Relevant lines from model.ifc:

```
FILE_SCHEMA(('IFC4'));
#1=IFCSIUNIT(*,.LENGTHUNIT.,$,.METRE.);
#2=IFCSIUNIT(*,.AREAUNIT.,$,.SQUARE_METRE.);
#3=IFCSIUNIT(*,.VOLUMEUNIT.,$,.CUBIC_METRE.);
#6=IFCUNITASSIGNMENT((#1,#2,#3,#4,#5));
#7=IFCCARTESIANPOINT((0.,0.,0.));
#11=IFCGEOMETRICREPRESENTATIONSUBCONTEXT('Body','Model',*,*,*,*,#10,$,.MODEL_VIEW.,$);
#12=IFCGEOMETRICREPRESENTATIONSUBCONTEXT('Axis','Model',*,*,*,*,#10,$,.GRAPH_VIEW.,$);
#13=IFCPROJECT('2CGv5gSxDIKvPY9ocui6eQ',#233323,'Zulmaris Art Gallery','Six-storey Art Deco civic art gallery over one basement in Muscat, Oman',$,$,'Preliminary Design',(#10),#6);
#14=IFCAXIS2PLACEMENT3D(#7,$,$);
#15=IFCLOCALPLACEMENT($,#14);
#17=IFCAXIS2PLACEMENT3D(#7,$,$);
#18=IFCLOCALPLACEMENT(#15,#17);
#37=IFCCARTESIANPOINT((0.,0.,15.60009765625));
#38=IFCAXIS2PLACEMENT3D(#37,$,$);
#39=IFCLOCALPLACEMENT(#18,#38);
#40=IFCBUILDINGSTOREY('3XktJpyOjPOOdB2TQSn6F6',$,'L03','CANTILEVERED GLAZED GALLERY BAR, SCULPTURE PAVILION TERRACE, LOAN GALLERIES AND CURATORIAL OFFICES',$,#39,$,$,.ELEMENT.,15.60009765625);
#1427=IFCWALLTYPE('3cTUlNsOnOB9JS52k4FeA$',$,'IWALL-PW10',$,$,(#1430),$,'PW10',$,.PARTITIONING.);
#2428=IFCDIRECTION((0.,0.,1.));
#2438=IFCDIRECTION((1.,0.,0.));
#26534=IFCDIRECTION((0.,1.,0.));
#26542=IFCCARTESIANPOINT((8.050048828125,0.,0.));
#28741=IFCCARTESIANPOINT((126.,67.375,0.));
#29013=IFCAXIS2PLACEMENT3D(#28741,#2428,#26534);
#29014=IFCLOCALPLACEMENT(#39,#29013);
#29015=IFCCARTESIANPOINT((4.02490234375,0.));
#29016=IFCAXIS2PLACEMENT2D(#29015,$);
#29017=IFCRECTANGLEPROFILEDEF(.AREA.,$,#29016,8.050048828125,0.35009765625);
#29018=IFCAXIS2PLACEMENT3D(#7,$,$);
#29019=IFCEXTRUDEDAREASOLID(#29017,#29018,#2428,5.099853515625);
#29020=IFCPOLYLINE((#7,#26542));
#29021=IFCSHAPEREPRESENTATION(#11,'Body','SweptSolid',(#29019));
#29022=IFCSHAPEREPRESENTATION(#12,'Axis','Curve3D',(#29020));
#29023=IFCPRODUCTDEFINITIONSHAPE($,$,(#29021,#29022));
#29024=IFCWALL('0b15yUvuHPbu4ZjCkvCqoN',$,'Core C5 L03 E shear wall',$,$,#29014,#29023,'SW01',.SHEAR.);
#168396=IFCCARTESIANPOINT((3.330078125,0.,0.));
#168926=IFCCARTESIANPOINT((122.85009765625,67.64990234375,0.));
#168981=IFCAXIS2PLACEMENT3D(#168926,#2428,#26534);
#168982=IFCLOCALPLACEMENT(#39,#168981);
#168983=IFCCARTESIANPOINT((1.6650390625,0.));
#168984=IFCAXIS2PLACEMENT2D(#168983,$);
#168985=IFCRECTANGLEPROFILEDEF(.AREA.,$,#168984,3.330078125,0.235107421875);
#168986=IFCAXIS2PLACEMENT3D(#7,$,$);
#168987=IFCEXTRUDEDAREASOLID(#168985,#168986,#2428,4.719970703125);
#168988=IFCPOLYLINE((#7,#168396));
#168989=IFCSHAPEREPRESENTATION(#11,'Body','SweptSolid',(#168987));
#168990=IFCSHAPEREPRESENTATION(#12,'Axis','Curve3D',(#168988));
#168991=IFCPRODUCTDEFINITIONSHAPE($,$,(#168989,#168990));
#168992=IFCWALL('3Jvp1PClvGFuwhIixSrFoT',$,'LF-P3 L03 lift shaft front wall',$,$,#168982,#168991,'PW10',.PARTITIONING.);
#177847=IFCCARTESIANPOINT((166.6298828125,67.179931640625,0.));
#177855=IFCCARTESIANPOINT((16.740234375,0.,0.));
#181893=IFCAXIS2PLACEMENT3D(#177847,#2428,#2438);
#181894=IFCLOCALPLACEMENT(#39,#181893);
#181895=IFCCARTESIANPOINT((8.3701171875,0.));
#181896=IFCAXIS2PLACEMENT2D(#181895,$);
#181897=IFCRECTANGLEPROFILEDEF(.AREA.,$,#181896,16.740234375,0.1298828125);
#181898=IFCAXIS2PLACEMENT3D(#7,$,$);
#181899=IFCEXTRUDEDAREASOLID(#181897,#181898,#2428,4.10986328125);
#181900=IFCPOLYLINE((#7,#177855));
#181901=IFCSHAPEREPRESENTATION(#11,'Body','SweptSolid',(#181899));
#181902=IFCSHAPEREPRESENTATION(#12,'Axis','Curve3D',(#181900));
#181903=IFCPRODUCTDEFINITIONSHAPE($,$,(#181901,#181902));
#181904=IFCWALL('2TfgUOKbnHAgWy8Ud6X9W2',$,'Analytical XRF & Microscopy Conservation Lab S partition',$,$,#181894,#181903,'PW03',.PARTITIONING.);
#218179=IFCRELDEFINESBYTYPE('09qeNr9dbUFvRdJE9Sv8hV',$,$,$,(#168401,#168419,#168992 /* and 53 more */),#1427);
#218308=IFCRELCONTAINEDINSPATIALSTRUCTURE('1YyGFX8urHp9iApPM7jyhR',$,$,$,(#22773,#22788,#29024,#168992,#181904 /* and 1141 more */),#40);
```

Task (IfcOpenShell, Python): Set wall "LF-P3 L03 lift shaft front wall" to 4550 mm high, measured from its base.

```python
import ifcopenshell
import ifcopenshell.geom
import ifcopenshell.util.representation
import ifcopenshell.util.shape
import ifcopenshell.util.unit

model = ifcopenshell.open("model.ifc")
unit_scale = ifcopenshell.util.unit.calculate_unit_scale(model)
settings = ifcopenshell.geom.settings()


def volume(element):
    """Net volume in cubic metres, openings subtracted."""
    shape = ifcopenshell.geom.create_shape(settings, element)
    return ifcopenshell.util.shape.get_volume(shape.geometry)


wall = model.by_guid("3Jvp1PClvGFuwhIixSrFoT")
before = volume(wall)

body = ifcopenshell.util.representation.get_representation(wall, "Model", "Body")
solid = body.Items[0]
old_height = solid.Depth
solid.Depth = 4.55 / unit_scale
after = volume(wall)

print(f"height {old_height:g} -> {solid.Depth:g}, volume {before:.3f} -> {after:.3f} m3")

model.write("model_rev.ifc")
```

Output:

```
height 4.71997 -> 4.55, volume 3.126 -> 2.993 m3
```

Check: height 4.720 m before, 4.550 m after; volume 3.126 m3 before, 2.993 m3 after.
